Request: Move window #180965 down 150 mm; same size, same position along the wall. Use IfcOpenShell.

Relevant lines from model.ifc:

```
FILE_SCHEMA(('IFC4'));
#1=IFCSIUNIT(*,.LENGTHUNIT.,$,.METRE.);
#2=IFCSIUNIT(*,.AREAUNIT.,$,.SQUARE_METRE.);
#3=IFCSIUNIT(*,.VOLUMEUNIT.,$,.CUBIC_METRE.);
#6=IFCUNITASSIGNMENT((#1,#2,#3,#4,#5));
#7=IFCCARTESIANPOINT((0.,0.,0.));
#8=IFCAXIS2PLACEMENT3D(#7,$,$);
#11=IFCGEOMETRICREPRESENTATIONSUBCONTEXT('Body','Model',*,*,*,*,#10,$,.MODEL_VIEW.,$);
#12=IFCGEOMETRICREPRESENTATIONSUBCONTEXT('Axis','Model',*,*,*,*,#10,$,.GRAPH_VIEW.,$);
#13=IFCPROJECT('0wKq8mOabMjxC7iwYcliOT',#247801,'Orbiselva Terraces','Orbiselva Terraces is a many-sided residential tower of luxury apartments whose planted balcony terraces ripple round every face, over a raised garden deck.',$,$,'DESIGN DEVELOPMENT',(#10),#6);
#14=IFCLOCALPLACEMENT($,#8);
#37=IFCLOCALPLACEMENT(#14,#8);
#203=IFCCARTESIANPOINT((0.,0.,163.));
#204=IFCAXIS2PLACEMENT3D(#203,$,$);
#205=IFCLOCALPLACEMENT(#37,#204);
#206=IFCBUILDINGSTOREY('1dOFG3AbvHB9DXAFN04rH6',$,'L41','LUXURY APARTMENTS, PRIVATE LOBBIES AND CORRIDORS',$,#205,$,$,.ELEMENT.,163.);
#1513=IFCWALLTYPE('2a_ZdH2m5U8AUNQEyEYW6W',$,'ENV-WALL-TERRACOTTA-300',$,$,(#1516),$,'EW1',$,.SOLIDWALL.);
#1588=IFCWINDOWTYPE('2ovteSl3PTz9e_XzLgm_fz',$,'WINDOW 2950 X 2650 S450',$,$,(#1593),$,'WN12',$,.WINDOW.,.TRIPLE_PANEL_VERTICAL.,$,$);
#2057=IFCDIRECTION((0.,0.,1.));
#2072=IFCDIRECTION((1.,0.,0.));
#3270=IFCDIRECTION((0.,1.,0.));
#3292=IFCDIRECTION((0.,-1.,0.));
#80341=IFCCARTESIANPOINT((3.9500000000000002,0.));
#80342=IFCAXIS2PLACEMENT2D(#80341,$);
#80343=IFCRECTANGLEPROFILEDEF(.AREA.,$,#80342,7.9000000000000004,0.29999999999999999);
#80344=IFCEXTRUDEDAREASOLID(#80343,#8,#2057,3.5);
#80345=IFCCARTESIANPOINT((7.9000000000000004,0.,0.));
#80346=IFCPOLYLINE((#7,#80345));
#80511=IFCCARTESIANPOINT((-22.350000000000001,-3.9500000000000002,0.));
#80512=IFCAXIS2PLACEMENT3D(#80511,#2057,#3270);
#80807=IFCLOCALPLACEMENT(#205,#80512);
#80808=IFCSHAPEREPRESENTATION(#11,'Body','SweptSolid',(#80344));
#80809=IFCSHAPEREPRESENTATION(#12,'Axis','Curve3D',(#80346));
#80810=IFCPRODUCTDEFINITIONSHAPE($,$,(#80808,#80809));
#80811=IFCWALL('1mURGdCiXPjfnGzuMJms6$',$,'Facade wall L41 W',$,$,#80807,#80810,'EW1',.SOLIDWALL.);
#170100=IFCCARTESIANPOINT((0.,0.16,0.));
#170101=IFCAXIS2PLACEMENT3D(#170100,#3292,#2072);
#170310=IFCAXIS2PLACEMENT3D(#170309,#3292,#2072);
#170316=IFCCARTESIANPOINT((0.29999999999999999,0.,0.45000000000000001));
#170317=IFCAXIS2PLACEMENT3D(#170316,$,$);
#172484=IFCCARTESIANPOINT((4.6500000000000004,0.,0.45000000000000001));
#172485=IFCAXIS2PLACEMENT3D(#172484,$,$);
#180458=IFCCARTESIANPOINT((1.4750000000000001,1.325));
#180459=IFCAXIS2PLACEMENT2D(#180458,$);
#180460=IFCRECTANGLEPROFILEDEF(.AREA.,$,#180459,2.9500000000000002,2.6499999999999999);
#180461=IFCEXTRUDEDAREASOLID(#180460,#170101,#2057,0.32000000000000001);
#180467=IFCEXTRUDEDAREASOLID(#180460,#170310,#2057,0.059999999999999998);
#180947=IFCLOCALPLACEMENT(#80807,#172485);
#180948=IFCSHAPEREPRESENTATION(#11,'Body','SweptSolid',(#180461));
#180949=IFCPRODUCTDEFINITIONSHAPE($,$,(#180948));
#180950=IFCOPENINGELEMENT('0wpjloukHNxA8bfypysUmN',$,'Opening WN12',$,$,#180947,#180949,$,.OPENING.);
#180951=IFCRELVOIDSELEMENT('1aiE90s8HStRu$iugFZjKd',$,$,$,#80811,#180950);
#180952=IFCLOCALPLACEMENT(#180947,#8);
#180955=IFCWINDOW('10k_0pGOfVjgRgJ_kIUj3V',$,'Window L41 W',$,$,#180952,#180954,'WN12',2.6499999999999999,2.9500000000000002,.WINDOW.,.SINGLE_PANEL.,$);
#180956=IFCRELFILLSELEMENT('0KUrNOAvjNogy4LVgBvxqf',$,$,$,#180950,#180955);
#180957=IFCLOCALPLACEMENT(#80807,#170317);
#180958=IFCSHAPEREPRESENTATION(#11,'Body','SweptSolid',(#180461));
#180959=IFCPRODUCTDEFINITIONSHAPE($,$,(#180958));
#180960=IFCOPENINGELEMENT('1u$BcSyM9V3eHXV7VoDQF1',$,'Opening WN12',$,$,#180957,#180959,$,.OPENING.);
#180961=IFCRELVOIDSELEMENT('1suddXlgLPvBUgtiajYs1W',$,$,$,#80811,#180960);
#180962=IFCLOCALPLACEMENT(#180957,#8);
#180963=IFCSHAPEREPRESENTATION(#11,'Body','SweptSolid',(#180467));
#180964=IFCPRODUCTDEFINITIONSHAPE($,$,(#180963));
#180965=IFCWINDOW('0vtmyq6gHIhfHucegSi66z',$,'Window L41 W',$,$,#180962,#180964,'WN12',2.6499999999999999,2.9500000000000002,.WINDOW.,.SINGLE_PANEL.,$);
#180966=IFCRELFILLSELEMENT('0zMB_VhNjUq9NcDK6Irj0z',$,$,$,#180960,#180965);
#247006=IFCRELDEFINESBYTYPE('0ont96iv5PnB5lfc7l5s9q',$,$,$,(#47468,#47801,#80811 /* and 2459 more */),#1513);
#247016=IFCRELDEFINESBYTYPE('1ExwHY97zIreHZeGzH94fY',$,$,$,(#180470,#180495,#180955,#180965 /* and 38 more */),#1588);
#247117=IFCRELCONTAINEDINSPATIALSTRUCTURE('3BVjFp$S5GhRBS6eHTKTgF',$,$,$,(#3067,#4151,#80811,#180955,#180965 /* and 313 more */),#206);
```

```python
import numpy as np
import ifcopenshell
import ifcopenshell.api.geometry
import ifcopenshell.util.placement
import ifcopenshell.util.unit

model = ifcopenshell.open("model.ifc")
unit_scale = ifcopenshell.util.unit.calculate_unit_scale(model)

window = model.by_id(180965)
opening = window.FillsVoids[0].RelatingOpeningElement
dz = -0.15

shift = np.array([0.0, 0.0, dz])
# The window is placed relative to its opening, so it follows when the opening moves.
matrix = ifcopenshell.util.placement.get_local_placement(opening.ObjectPlacement)
matrix[:3, 3] += shift
ifcopenshell.api.geometry.edit_object_placement(
    model, product=opening, matrix=matrix, is_si=False, should_transform_children=True
)

print(f"moved by {dz * unit_scale:+.3f} m")

model.write("model-out.ifc")
```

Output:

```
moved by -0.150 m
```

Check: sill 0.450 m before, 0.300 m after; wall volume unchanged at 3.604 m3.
